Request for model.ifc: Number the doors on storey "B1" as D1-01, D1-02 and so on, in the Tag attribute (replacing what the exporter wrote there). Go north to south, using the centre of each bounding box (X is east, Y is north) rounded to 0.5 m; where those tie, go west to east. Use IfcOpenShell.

First a look at what the model holds.

```python
import ifcopenshell
import ifcopenshell.util.element
import ifcopenshell.util.placement

model = ifcopenshell.open("model.ifc")
print(model.schema)
storey = next(s for s in model.by_type("IfcBuildingStorey") if s.Name == "B1")
doors = [e for e in ifcopenshell.util.element.get_decomposition(storey) if e.is_a("IfcDoor")]
for e in sorted(doors, key=lambda e: e.id()):
    origin = ifcopenshell.util.placement.get_local_placement(e.ObjectPlacement)[:3, 3]
    print(e.id(), e.Tag, e.Name, origin.round(2) + 0.0, sep=" | ")
```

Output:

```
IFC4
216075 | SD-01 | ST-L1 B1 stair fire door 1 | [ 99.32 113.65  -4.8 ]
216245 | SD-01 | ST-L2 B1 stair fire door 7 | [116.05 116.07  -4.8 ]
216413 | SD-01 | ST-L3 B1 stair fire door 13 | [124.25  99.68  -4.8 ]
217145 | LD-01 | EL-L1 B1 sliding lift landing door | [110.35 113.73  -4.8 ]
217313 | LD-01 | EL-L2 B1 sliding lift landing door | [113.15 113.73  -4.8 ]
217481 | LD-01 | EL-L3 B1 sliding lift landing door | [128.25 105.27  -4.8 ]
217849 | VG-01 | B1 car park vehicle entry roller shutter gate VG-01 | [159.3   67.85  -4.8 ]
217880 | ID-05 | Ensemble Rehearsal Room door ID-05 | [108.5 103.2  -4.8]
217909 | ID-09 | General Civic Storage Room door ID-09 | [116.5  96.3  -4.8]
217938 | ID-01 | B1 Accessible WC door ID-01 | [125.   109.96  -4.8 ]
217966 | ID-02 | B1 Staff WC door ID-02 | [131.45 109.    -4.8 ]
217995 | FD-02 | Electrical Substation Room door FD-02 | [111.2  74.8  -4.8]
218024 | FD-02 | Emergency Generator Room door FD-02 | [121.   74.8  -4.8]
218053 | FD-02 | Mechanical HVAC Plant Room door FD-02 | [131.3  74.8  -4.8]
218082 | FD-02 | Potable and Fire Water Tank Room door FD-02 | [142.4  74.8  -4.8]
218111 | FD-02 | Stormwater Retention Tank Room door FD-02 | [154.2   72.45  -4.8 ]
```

```python
import ifcopenshell
import ifcopenshell.geom
import ifcopenshell.util.element
import ifcopenshell.util.shape

model = ifcopenshell.open("model.ifc")
settings = ifcopenshell.geom.settings()
settings.set("use-world-coords", True)


def centre(element):
    shape = ifcopenshell.geom.create_shape(settings, element)
    return ifcopenshell.util.shape.get_bbox_centroid(shape.geometry)


storey = next(s for s in model.by_type("IfcBuildingStorey") if s.Name == "B1")
doors = [e for e in ifcopenshell.util.element.get_decomposition(storey) if e.is_a("IfcDoor")]

# Insertion points can sit at a corner or the storey origin, so sort by the geometry (in metres).
centres = {e: centre(e) for e in doors}
doors.sort(key=lambda e: (-round(centres[e][1] / 0.5), centres[e][0]))

for i, e in enumerate(doors, start=1):
    number = f"D1-{i:02d}"
    e.Tag = number
    print(e.id(), number)

model.write("model_edited.ifc")
```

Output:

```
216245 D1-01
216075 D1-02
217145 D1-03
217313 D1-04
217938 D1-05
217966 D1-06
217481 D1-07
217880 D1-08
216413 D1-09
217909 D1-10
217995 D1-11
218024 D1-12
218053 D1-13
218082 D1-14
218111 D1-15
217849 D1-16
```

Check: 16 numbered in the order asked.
